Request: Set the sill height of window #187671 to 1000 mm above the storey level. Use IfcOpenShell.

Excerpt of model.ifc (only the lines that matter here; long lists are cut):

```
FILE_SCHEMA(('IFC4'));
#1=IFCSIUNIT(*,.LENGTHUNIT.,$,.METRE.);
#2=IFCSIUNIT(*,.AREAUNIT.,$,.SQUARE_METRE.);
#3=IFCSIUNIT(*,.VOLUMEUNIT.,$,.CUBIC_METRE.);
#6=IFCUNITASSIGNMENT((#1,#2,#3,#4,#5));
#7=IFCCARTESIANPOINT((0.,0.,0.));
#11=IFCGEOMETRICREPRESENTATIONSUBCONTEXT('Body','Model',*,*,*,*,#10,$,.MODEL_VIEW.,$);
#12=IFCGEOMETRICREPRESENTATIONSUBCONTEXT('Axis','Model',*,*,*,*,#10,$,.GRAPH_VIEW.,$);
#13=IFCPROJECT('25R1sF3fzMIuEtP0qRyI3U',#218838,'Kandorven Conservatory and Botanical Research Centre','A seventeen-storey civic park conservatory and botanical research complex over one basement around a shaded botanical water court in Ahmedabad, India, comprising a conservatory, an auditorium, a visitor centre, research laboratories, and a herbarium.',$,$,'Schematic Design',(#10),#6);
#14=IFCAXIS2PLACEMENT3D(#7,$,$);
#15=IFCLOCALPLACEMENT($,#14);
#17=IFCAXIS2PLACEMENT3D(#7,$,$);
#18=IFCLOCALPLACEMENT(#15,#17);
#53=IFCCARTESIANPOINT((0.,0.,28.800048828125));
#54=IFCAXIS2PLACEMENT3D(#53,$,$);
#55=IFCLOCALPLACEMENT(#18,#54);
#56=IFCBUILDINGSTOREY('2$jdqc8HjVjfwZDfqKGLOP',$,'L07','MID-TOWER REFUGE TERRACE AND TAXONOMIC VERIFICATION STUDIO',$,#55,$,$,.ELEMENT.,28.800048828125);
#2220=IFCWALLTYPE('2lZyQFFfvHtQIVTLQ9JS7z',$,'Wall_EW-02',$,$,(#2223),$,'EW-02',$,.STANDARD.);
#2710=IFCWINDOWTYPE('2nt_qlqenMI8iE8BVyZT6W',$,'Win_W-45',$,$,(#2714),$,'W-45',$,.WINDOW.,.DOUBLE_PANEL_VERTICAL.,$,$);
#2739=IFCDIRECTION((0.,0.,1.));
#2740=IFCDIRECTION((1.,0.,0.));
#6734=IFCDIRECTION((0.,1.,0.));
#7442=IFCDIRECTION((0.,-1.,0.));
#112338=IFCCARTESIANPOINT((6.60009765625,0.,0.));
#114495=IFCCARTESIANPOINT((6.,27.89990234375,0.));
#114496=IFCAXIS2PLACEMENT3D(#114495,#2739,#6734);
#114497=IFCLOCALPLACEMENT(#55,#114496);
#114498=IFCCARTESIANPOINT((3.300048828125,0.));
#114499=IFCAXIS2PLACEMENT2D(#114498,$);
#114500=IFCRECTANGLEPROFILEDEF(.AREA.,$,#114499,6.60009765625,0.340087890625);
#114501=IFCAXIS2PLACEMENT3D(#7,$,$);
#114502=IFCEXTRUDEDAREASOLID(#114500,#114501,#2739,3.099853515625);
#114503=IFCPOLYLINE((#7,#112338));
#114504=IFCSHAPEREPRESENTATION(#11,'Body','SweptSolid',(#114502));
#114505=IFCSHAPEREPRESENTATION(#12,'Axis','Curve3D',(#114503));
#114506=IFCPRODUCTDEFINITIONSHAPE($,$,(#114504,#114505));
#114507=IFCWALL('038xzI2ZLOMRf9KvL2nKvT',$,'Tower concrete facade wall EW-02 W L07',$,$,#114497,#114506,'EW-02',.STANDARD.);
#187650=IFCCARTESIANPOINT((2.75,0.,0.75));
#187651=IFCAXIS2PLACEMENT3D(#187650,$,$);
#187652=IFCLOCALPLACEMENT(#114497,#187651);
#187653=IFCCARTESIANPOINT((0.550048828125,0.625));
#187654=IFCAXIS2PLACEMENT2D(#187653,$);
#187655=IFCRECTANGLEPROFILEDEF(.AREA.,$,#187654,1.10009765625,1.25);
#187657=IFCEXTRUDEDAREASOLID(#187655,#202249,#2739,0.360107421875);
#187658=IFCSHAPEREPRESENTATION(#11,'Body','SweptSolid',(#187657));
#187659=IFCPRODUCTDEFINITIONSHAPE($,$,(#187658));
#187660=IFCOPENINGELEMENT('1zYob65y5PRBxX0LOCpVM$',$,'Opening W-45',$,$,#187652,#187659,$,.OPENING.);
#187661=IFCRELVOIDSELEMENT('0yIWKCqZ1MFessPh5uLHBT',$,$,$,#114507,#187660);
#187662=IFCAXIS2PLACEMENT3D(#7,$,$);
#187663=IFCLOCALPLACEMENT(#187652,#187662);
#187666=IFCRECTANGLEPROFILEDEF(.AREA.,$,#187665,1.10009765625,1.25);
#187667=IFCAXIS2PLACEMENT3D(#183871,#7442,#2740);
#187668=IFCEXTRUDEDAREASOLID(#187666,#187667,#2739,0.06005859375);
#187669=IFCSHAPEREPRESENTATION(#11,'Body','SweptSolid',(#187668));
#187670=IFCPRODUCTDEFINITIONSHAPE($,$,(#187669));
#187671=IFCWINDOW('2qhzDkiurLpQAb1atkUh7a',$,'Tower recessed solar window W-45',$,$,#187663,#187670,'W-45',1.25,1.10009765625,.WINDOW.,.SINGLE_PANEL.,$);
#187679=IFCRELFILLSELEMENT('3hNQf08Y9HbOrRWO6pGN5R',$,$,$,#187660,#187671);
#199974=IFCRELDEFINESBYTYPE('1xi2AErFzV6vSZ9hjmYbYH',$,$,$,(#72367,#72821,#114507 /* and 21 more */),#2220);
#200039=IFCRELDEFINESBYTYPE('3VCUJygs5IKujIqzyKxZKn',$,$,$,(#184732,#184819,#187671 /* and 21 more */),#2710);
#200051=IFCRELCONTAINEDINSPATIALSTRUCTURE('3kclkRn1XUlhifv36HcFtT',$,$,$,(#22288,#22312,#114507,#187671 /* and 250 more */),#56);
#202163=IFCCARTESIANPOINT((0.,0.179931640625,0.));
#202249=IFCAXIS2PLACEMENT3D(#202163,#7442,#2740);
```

```python
import numpy as np
import ifcopenshell
import ifcopenshell.api.geometry
import ifcopenshell.geom
import ifcopenshell.util.element
import ifcopenshell.util.placement
import ifcopenshell.util.shape
import ifcopenshell.util.unit

model = ifcopenshell.open("model.ifc")
unit_scale = ifcopenshell.util.unit.calculate_unit_scale(model)

window = model.by_id(187671)
opening = window.FillsVoids[0].RelatingOpeningElement
storey = ifcopenshell.util.element.get_container(window, ifc_class="IfcBuildingStorey")
level = ifcopenshell.util.placement.get_local_placement(storey.ObjectPlacement)[2, 3]

# The opening's origin need not be at the sill, so measure its lowest point.
shape = ifcopenshell.geom.create_shape(ifcopenshell.geom.settings(), opening)
bottom = ifcopenshell.util.shape.get_shape_bottom_elevation(shape, shape.geometry) / unit_scale
dz = level + 1.0 - bottom

shift = np.array([0.0, 0.0, dz])
# The window is placed relative to its opening, so it follows when the opening moves.
matrix = ifcopenshell.util.placement.get_local_placement(opening.ObjectPlacement)
matrix[:3, 3] += shift
ifcopenshell.api.geometry.edit_object_placement(
    model, product=opening, matrix=matrix, is_si=False, should_transform_children=True
)

print(f"moved by {dz * unit_scale:+.3f} m")

model.write("model-out.ifc")
```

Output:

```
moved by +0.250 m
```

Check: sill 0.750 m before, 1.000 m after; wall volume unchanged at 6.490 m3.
